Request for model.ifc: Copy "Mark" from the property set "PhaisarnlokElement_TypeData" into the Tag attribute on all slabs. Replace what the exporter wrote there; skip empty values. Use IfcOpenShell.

First a look at what the model holds.

```python
import ifcopenshell
import ifcopenshell.util.element

model = ifcopenshell.open("model.ifc")
print(model.schema)
slabs = model.by_type("IfcSlab")
print(len(slabs), "slabs")
for e in slabs[:8]:
    source = ifcopenshell.util.element.get_pset(e, "PhaisarnlokElement_TypeData", "Mark")
    target = e.Tag
    print(e.id(), repr(source), repr(target), sep=" | ")
```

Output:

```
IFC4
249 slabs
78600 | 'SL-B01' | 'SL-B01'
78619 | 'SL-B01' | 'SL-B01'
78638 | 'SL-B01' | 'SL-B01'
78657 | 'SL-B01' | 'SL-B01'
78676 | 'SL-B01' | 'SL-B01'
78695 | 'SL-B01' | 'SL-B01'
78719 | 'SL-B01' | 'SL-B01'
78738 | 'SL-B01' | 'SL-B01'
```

```python
import ifcopenshell
import ifcopenshell.util.element

model = ifcopenshell.open("model.ifc")

count = 0
for e in model.by_type("IfcSlab"):
    value = ifcopenshell.util.element.get_pset(e, "PhaisarnlokElement_TypeData", "Mark")
    current = e.Tag
    if not value or not value.strip() or current == value:
        continue
    e.Tag = value
    count += 1

print(count, "slabs updated")

model.write("model_edited.ifc")
```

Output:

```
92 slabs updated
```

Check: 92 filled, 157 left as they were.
